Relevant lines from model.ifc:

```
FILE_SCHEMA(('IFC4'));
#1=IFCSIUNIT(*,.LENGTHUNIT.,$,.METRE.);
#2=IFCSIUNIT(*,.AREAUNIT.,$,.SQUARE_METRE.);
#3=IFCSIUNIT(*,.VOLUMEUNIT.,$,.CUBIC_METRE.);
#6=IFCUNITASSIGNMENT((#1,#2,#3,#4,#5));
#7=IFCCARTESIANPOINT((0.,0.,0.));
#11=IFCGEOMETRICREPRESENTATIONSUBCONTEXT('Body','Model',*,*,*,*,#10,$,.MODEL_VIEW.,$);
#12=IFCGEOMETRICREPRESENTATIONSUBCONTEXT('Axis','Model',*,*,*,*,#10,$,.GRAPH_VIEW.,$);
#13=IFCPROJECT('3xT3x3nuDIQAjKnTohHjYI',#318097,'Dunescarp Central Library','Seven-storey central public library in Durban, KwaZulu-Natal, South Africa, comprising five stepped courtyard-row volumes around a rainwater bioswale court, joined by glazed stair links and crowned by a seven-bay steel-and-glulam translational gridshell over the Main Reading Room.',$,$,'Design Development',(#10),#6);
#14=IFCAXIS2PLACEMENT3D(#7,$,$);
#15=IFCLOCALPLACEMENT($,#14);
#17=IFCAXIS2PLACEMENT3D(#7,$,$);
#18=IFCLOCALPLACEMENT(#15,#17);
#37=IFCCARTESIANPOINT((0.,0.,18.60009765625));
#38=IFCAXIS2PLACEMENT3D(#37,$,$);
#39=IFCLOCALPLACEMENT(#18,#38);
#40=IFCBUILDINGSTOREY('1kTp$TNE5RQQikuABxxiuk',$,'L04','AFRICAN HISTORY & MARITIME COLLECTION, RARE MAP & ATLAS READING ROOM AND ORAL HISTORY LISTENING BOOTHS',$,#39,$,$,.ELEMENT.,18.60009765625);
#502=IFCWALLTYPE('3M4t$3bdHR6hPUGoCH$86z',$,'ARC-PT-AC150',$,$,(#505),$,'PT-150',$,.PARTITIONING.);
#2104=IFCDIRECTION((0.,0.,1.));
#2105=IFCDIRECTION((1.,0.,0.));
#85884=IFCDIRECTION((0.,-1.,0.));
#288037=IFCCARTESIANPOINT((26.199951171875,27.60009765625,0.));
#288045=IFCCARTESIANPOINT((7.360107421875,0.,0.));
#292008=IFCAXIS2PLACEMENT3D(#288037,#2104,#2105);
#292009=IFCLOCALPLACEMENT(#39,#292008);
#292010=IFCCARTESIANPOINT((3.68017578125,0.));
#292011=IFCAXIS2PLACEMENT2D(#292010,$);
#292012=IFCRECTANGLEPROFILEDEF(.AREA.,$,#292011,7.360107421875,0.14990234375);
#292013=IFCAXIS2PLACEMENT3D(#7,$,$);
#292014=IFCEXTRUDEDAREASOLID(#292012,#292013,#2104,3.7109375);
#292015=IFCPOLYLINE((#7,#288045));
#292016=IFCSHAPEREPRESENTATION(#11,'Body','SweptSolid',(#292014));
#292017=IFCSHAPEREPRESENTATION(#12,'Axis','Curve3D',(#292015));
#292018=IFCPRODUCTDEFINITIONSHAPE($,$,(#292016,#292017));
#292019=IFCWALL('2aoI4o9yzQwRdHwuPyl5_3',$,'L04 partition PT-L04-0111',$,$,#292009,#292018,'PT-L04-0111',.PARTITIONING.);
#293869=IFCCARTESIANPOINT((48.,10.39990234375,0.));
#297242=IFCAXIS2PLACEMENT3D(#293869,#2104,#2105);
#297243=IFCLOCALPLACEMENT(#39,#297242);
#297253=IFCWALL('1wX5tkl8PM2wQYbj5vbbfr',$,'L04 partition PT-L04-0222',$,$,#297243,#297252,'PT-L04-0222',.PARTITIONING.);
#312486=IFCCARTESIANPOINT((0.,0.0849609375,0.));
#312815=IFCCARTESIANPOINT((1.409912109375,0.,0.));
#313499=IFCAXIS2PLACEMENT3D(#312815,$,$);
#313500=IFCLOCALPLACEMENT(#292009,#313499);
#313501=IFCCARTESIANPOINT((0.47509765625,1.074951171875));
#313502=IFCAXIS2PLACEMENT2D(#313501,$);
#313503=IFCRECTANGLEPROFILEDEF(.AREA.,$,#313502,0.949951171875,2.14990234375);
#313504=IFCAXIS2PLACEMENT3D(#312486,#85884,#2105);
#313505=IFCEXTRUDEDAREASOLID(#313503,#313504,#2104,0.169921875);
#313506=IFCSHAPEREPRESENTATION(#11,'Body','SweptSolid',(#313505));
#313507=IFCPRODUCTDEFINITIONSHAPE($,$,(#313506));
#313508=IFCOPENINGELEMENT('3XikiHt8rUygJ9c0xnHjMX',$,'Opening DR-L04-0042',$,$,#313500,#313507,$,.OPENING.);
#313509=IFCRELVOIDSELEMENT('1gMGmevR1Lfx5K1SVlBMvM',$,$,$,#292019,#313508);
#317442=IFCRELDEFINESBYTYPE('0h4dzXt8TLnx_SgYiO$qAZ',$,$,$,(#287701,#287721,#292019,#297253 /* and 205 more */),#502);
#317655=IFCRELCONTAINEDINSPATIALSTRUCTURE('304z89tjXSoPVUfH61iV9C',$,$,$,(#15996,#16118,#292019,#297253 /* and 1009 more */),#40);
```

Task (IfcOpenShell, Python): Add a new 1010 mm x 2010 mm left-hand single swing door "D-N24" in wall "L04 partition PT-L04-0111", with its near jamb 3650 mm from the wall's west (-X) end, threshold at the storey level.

```python
import numpy as np
import ifcopenshell
import ifcopenshell.api.feature
import ifcopenshell.api.geometry
import ifcopenshell.api.root
import ifcopenshell.api.spatial
import ifcopenshell.geom
import ifcopenshell.util.element
import ifcopenshell.util.placement
import ifcopenshell.util.representation
import ifcopenshell.util.shape
import ifcopenshell.util.unit

model = ifcopenshell.open("model.ifc")
unit_scale = ifcopenshell.util.unit.calculate_unit_scale(model)
settings = ifcopenshell.geom.settings()


def volume(element):
    """Net volume in cubic metres, openings subtracted."""
    shape = ifcopenshell.geom.create_shape(settings, element)
    return ifcopenshell.util.shape.get_volume(shape.geometry)


wall = model.by_guid("2aoI4o9yzQwRdHwuPyl5_3")
storey = ifcopenshell.util.element.get_container(wall, ifc_class="IfcBuildingStorey")
context = ifcopenshell.util.representation.get_context(model, "Model", "Body", "MODEL_VIEW")
before = volume(wall)

width, height, from_end, sill = 1.01, 2.01, 3.65, 0.0  # metres

# The wall runs along its own X axis, and the end named is its -X end.
wall_shape = ifcopenshell.geom.create_shape(settings, wall)
x, y, z = ifcopenshell.util.shape.get_vertices(wall_shape.geometry).T
start = x.min() + from_end
face, thickness = float(y.min()), float(y.max() - y.min())
wall_matrix = ifcopenshell.util.placement.get_local_placement(wall.ObjectPlacement)
level = ifcopenshell.util.placement.get_local_placement(storey.ObjectPlacement)[2, 3]


def in_wall(x, y):
    """Placement at x, y metres in the wall's axes, at sill height."""
    matrix = wall_matrix.copy()
    matrix[:, 3] = wall_matrix @ np.array([x / unit_scale, y / unit_scale, 0.0, 1.0])
    matrix[2, 3] = level + sill / unit_scale
    return matrix


# Opening: a box that overshoots both wall faces by 50 mm.
opening = ifcopenshell.api.root.create_entity(model, ifc_class="IfcOpeningElement", predefined_type="OPENING")
box = ifcopenshell.api.geometry.add_wall_representation(
    model, context=context, length=width, height=height, thickness=thickness + 0.1
)
ifcopenshell.api.geometry.assign_representation(model, product=opening, representation=box)
ifcopenshell.api.geometry.edit_object_placement(model, product=opening, matrix=in_wall(start, face - 0.05), is_si=False)
ifcopenshell.api.feature.add_feature(model, feature=opening, element=wall)

door = ifcopenshell.api.root.create_entity(model, ifc_class="IfcDoor", name="D-N24", predefined_type="DOOR")
door.OverallWidth, door.OverallHeight = width / unit_scale, height / unit_scale
door.OperationType = "SINGLE_SWING_LEFT"
body = ifcopenshell.api.geometry.add_door_representation(
    model,
    context=context,
    overall_width=door.OverallWidth,
    overall_height=door.OverallHeight,
    operation_type="SINGLE_SWING_LEFT",
    lining_properties={"LiningDepth": thickness / unit_scale, "ThresholdDepth": thickness / unit_scale},
)
ifcopenshell.api.geometry.assign_representation(model, product=door, representation=body)
ifcopenshell.api.spatial.assign_container(model, products=[door], relating_structure=storey)
ifcopenshell.api.feature.add_filling(model, opening=opening, element=door)

# The lining spans the wall, so the door starts at the wall face.
ifcopenshell.api.geometry.edit_object_placement(model, product=door, matrix=in_wall(start, face), is_si=False)

after = volume(wall)

print(f"wall volume {before:.3f} -> {after:.3f} m3")

model.write("model_updated.ifc")
```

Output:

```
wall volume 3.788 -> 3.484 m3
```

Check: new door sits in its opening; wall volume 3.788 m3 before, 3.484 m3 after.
